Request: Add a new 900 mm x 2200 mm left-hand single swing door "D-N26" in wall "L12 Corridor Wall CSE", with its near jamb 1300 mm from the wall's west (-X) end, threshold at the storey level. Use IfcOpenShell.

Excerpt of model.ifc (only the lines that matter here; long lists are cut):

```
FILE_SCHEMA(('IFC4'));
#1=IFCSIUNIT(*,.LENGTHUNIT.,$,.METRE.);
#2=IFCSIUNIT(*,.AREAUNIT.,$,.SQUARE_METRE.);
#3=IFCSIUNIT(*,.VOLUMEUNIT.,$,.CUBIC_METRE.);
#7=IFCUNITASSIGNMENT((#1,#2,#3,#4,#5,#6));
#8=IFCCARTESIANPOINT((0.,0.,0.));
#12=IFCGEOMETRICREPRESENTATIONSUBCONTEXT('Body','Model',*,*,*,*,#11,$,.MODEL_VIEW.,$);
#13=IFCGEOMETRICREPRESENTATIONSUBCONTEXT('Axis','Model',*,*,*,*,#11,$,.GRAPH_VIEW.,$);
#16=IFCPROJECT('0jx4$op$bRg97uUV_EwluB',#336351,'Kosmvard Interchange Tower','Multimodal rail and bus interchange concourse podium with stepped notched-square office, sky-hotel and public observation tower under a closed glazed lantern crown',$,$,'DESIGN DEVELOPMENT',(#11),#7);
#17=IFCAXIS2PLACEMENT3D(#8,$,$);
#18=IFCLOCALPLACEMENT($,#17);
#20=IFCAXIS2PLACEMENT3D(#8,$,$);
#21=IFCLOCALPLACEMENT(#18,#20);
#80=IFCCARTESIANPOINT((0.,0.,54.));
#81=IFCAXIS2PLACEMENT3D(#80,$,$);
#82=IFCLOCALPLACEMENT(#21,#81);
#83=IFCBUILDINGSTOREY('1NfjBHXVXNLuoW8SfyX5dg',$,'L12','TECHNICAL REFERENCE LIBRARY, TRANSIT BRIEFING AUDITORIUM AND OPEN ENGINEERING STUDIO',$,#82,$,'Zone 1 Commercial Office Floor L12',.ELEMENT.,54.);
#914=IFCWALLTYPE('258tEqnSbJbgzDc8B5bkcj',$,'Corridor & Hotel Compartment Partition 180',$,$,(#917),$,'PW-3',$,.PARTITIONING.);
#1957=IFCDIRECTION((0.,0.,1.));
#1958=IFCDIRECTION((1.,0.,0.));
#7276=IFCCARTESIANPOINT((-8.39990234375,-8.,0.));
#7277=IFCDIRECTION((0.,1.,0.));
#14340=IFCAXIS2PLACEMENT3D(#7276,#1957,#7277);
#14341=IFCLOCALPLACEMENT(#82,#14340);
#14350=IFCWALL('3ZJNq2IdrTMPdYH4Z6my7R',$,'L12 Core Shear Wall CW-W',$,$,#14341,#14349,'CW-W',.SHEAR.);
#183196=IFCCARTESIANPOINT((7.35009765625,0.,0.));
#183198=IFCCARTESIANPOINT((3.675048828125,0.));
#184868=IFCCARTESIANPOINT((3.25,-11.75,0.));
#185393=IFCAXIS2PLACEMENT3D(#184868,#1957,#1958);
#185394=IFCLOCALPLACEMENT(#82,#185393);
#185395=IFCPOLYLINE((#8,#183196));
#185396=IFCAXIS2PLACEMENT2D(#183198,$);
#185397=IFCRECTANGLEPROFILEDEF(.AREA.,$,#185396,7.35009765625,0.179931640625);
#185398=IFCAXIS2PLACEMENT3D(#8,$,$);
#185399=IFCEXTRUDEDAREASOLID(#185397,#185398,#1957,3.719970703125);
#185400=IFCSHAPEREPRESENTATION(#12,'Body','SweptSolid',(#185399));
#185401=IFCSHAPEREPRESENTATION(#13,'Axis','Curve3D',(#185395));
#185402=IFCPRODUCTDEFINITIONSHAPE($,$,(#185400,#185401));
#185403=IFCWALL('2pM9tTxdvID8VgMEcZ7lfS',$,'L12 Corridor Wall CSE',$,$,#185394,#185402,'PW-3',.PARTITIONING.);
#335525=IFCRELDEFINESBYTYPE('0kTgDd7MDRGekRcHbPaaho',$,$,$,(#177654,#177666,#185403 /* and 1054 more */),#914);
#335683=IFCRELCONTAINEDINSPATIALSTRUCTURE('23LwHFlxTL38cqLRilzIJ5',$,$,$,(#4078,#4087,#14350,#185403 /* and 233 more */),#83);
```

```python
import numpy as np
import ifcopenshell
import ifcopenshell.api.feature
import ifcopenshell.api.geometry
import ifcopenshell.api.root
import ifcopenshell.api.spatial
import ifcopenshell.geom
import ifcopenshell.util.element
import ifcopenshell.util.placement
import ifcopenshell.util.representation
import ifcopenshell.util.shape
import ifcopenshell.util.unit

model = ifcopenshell.open("model.ifc")
unit_scale = ifcopenshell.util.unit.calculate_unit_scale(model)
settings = ifcopenshell.geom.settings()


def volume(element):
    """Net volume in cubic metres, openings subtracted."""
    shape = ifcopenshell.geom.create_shape(settings, element)
    return ifcopenshell.util.shape.get_volume(shape.geometry)


wall = model.by_guid("2pM9tTxdvID8VgMEcZ7lfS")
storey = ifcopenshell.util.element.get_container(wall, ifc_class="IfcBuildingStorey")
context = ifcopenshell.util.representation.get_context(model, "Model", "Body", "MODEL_VIEW")
before = volume(wall)

width, height, from_end, sill = 0.9, 2.2, 1.3, 0.0  # metres

# The wall runs along its own X axis, and the end named is its -X end.
wall_shape = ifcopenshell.geom.create_shape(settings, wall)
x, y, z = ifcopenshell.util.shape.get_vertices(wall_shape.geometry).T
start = x.min() + from_end
face, thickness = float(y.min()), float(y.max() - y.min())
wall_matrix = ifcopenshell.util.placement.get_local_placement(wall.ObjectPlacement)
level = ifcopenshell.util.placement.get_local_placement(storey.ObjectPlacement)[2, 3]


def in_wall(x, y):
    """Placement at x, y metres in the wall's axes, at sill height."""
    matrix = wall_matrix.copy()
    matrix[:, 3] = wall_matrix @ np.array([x / unit_scale, y / unit_scale, 0.0, 1.0])
    matrix[2, 3] = level + sill / unit_scale
    return matrix


# Opening: a box that overshoots both wall faces by 50 mm.
opening = ifcopenshell.api.root.create_entity(model, ifc_class="IfcOpeningElement", predefined_type="OPENING")
box = ifcopenshell.api.geometry.add_wall_representation(
    model, context=context, length=width, height=height, thickness=thickness + 0.1
)
ifcopenshell.api.geometry.assign_representation(model, product=opening, representation=box)
ifcopenshell.api.geometry.edit_object_placement(model, product=opening, matrix=in_wall(start, face - 0.05), is_si=False)
ifcopenshell.api.feature.add_feature(model, feature=opening, element=wall)

door = ifcopenshell.api.root.create_entity(model, ifc_class="IfcDoor", name="D-N26", predefined_type="DOOR")
door.OverallWidth, door.OverallHeight = width / unit_scale, height / unit_scale
door.OperationType = "SINGLE_SWING_LEFT"
body = ifcopenshell.api.geometry.add_door_representation(
    model,
    context=context,
    overall_width=door.OverallWidth,
    overall_height=door.OverallHeight,
    operation_type="SINGLE_SWING_LEFT",
    lining_properties={"LiningDepth": thickness / unit_scale, "ThresholdDepth": thickness / unit_scale},
)
ifcopenshell.api.geometry.assign_representation(model, product=door, representation=body)
ifcopenshell.api.spatial.assign_container(model, products=[door], relating_structure=storey)
ifcopenshell.api.feature.add_filling(model, opening=opening, element=door)

# The lining spans the wall, so the door starts at the wall face.
ifcopenshell.api.geometry.edit_object_placement(model, product=door, matrix=in_wall(start, face), is_si=False)

after = volume(wall)

print(f"wall volume {before:.3f} -> {after:.3f} m3")

model.write("model-out.ifc")
```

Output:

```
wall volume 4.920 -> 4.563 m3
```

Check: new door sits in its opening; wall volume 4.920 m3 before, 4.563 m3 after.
